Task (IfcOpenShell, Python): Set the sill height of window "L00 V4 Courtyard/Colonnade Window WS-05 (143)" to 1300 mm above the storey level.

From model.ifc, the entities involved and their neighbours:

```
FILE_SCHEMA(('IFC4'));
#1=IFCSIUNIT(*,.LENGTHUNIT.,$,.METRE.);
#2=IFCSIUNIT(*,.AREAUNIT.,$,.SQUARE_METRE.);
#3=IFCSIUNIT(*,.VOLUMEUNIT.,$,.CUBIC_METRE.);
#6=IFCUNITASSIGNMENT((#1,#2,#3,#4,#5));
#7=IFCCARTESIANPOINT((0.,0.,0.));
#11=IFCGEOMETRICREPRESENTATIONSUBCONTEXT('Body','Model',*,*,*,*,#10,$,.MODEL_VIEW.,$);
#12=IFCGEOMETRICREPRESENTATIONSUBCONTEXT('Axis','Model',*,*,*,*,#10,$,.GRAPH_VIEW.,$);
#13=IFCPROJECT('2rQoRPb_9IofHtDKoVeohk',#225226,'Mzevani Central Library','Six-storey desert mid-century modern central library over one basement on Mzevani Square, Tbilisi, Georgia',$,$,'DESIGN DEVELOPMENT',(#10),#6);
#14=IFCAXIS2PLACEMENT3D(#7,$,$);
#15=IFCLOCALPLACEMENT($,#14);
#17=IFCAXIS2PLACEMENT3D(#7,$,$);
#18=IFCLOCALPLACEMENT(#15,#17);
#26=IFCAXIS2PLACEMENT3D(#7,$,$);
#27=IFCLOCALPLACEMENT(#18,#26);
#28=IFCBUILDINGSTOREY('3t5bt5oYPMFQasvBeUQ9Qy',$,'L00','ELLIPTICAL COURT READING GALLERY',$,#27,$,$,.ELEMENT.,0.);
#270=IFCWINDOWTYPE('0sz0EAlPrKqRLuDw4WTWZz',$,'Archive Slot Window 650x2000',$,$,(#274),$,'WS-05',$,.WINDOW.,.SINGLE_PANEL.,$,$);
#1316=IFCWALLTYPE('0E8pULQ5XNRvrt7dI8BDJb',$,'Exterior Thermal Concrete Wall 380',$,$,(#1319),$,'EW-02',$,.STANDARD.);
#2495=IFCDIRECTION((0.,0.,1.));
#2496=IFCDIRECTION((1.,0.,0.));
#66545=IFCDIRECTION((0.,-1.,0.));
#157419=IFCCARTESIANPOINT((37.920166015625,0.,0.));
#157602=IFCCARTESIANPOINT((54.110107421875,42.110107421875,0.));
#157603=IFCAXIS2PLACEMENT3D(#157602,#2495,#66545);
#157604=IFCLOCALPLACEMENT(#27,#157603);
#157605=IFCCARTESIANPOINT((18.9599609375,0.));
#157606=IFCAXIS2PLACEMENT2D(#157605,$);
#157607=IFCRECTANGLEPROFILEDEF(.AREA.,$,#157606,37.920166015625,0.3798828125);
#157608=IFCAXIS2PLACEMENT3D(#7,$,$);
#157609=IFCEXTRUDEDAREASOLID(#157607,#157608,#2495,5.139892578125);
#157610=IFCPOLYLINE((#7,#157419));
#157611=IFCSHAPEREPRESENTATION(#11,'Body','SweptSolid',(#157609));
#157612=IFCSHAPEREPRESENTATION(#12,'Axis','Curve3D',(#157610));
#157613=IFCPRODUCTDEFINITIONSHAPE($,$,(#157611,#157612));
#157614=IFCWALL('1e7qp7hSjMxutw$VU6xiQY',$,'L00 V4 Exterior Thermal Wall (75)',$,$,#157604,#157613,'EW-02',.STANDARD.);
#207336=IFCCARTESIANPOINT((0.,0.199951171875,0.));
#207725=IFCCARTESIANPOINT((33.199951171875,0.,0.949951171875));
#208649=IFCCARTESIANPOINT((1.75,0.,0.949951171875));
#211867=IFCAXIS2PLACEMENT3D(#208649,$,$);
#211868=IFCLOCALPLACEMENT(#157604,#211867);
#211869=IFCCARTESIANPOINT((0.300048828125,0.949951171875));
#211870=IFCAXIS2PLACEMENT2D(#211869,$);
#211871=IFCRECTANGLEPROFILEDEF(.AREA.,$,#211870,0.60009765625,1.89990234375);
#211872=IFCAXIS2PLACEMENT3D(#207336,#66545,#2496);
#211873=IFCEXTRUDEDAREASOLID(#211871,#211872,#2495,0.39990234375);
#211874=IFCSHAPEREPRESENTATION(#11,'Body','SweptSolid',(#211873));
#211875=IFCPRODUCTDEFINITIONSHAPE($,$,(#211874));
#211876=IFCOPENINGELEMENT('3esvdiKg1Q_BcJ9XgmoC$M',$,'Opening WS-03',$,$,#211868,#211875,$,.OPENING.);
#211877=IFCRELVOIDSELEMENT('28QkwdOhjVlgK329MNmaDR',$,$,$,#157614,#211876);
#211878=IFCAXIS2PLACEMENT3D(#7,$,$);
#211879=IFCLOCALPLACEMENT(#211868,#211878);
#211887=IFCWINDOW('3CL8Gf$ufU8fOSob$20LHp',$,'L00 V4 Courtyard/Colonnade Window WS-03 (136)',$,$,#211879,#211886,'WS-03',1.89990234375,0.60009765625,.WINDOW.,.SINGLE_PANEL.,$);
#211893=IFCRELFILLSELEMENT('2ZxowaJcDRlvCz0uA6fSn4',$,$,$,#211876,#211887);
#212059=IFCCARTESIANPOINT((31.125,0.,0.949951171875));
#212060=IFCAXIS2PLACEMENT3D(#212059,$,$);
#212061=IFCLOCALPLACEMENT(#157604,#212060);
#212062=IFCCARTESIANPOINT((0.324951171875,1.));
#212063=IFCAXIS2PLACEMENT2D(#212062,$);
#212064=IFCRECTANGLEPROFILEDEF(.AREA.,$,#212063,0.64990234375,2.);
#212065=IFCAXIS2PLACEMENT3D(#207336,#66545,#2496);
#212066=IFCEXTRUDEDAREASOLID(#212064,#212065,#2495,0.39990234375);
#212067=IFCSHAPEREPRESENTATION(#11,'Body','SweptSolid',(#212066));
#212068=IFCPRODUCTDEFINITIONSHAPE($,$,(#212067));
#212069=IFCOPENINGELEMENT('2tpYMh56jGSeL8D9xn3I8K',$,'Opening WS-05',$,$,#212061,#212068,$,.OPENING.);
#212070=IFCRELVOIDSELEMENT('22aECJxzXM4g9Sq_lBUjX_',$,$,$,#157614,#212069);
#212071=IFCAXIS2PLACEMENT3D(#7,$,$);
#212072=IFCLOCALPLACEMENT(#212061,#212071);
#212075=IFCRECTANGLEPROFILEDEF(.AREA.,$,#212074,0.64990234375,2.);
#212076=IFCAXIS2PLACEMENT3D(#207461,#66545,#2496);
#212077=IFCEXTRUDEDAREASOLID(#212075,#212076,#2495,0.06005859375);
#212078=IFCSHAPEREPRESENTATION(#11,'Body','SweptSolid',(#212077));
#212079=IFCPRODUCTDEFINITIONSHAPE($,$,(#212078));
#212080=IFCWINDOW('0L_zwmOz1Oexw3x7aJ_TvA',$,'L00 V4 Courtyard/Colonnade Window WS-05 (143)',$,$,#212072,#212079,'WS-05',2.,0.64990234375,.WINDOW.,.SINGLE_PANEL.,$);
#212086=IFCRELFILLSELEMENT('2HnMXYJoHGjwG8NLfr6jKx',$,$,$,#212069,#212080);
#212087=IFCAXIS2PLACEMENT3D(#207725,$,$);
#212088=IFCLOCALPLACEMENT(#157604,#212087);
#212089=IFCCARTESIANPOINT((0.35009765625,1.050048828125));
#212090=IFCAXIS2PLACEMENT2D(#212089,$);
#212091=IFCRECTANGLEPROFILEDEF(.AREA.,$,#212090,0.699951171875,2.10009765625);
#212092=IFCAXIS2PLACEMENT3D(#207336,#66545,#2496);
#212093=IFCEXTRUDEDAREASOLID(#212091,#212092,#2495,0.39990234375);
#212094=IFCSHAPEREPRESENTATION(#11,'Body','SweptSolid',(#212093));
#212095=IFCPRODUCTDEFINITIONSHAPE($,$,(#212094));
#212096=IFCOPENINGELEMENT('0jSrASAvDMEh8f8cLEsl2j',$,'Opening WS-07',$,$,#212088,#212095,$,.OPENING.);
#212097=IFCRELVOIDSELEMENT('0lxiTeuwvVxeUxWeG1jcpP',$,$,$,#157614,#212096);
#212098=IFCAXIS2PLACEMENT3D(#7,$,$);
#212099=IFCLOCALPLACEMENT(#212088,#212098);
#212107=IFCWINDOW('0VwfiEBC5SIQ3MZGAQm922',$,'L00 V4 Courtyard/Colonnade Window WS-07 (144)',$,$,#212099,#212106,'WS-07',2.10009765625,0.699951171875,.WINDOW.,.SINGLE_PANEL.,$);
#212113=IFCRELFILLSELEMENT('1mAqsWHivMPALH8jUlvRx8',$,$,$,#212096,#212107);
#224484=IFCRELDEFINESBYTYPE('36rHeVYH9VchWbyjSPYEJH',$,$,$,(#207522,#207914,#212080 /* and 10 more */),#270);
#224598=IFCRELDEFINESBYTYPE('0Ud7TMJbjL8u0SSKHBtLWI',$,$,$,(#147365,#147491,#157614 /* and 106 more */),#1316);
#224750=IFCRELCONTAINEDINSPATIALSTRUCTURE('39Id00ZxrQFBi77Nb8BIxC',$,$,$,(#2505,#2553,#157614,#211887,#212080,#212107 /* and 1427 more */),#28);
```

```python
import numpy as np
import ifcopenshell
import ifcopenshell.api.geometry
import ifcopenshell.geom
import ifcopenshell.util.element
import ifcopenshell.util.placement
import ifcopenshell.util.shape
import ifcopenshell.util.unit

model = ifcopenshell.open("model.ifc")
unit_scale = ifcopenshell.util.unit.calculate_unit_scale(model)

window = model.by_guid("0L_zwmOz1Oexw3x7aJ_TvA")
opening = window.FillsVoids[0].RelatingOpeningElement
storey = ifcopenshell.util.element.get_container(window, ifc_class="IfcBuildingStorey")
level = ifcopenshell.util.placement.get_local_placement(storey.ObjectPlacement)[2, 3]

# The opening's origin need not be at the sill, so measure its lowest point.
shape = ifcopenshell.geom.create_shape(ifcopenshell.geom.settings(), opening)
bottom = ifcopenshell.util.shape.get_shape_bottom_elevation(shape, shape.geometry) / unit_scale
dz = level + 1.3 - bottom

shift = np.array([0.0, 0.0, dz])
# The window is placed relative to its opening, so it follows when the opening moves.
matrix = ifcopenshell.util.placement.get_local_placement(opening.ObjectPlacement)
matrix[:3, 3] += shift
ifcopenshell.api.geometry.edit_object_placement(
    model, product=opening, matrix=matrix, is_si=False, should_transform_children=True
)

print(f"moved by {dz * unit_scale:+.3f} m")

model.write("model-out.ifc")
```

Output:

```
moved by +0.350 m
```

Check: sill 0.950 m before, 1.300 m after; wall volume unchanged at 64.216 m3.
